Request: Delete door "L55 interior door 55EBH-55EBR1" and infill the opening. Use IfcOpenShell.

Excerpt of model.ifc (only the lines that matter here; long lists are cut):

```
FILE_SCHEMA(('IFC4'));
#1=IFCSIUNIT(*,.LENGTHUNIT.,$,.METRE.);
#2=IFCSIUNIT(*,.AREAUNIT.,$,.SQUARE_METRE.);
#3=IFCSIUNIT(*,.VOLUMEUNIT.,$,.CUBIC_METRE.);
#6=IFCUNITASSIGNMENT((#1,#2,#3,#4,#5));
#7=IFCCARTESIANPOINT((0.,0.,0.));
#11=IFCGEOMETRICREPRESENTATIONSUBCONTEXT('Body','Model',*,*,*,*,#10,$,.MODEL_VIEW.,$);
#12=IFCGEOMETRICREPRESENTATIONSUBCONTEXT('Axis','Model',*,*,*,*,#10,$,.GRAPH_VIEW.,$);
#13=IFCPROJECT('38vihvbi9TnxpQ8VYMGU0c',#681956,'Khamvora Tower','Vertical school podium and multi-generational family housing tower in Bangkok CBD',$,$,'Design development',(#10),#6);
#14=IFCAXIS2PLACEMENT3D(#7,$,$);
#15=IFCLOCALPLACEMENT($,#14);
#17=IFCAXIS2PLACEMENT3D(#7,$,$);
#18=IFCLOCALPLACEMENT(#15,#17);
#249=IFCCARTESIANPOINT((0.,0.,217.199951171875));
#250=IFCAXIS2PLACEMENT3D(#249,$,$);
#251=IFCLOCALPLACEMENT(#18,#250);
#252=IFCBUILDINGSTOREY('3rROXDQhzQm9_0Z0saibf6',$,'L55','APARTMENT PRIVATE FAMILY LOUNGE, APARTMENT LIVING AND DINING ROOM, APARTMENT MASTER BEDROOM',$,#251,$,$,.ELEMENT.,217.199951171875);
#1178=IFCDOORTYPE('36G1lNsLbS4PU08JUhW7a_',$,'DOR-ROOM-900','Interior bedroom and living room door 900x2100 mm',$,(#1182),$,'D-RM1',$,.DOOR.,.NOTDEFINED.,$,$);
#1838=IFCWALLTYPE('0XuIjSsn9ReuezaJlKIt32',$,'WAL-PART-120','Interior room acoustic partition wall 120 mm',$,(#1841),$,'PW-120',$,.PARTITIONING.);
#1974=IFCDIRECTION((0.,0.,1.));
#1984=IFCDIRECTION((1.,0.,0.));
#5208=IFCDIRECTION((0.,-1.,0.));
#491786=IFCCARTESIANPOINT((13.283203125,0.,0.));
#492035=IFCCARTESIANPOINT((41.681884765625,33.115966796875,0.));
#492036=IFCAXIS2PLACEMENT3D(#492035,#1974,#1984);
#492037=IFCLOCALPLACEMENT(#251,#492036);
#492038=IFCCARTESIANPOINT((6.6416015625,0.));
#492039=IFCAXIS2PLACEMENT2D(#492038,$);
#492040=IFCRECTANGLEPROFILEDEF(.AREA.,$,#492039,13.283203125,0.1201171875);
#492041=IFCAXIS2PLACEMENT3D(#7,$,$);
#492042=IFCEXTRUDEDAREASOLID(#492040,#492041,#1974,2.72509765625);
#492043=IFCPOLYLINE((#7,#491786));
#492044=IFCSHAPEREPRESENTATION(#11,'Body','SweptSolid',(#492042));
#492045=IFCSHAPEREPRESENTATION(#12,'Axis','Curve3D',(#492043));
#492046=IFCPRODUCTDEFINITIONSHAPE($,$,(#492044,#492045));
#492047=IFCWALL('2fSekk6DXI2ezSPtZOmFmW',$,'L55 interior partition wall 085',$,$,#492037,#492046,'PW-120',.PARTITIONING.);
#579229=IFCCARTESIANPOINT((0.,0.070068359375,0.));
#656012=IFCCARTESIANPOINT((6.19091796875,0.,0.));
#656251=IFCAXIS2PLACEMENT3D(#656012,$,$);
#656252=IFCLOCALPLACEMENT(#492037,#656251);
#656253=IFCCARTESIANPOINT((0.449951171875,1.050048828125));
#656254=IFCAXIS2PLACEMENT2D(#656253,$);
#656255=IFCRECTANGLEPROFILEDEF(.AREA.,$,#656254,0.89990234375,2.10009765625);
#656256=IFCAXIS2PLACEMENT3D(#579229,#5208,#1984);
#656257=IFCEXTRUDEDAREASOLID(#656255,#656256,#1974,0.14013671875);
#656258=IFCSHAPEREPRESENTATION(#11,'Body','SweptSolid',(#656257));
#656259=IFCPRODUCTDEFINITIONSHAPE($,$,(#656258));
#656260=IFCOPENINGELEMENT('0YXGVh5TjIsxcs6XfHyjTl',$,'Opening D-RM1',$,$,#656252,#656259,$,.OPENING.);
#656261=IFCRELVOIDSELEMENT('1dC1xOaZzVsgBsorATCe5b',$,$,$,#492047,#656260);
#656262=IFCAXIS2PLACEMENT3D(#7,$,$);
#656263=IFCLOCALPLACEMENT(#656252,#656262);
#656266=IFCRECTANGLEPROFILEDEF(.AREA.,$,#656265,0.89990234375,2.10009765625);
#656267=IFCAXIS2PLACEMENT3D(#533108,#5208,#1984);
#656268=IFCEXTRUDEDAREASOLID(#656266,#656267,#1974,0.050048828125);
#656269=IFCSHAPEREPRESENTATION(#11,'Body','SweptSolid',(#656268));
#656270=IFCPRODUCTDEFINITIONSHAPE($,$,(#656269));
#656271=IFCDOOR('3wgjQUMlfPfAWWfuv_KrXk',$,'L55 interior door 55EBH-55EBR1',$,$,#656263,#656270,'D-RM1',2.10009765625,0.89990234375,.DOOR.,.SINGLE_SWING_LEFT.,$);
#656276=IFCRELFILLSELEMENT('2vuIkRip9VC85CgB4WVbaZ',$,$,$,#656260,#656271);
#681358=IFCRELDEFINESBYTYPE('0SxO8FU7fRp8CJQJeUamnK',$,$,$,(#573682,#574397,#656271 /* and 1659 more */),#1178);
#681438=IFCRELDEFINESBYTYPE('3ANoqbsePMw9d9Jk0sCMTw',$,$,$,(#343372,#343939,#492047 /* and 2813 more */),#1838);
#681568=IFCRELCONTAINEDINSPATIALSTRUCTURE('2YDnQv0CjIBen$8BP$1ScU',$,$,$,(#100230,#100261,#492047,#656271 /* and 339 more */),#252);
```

```python
import ifcopenshell
import ifcopenshell.api.feature
import ifcopenshell.api.root
import ifcopenshell.geom
import ifcopenshell.util.shape

model = ifcopenshell.open("model.ifc")
settings = ifcopenshell.geom.settings()


def volume(element):
    """Net volume in cubic metres, openings subtracted."""
    shape = ifcopenshell.geom.create_shape(settings, element)
    return ifcopenshell.util.shape.get_volume(shape.geometry)


door = model.by_guid("3wgjQUMlfPfAWWfuv_KrXk")
opening = door.FillsVoids[0].RelatingOpeningElement
wall = opening.VoidsElements[0].RelatingBuildingElement
before = volume(wall)

ifcopenshell.api.root.remove_product(model, product=door)
ifcopenshell.api.feature.remove_feature(model, feature=opening)

after = volume(wall)

print(f"wall volume {before:.3f} -> {after:.3f} m3")

model.write("model-out.ifc")
```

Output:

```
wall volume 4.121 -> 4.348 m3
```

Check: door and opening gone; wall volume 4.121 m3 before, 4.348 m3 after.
